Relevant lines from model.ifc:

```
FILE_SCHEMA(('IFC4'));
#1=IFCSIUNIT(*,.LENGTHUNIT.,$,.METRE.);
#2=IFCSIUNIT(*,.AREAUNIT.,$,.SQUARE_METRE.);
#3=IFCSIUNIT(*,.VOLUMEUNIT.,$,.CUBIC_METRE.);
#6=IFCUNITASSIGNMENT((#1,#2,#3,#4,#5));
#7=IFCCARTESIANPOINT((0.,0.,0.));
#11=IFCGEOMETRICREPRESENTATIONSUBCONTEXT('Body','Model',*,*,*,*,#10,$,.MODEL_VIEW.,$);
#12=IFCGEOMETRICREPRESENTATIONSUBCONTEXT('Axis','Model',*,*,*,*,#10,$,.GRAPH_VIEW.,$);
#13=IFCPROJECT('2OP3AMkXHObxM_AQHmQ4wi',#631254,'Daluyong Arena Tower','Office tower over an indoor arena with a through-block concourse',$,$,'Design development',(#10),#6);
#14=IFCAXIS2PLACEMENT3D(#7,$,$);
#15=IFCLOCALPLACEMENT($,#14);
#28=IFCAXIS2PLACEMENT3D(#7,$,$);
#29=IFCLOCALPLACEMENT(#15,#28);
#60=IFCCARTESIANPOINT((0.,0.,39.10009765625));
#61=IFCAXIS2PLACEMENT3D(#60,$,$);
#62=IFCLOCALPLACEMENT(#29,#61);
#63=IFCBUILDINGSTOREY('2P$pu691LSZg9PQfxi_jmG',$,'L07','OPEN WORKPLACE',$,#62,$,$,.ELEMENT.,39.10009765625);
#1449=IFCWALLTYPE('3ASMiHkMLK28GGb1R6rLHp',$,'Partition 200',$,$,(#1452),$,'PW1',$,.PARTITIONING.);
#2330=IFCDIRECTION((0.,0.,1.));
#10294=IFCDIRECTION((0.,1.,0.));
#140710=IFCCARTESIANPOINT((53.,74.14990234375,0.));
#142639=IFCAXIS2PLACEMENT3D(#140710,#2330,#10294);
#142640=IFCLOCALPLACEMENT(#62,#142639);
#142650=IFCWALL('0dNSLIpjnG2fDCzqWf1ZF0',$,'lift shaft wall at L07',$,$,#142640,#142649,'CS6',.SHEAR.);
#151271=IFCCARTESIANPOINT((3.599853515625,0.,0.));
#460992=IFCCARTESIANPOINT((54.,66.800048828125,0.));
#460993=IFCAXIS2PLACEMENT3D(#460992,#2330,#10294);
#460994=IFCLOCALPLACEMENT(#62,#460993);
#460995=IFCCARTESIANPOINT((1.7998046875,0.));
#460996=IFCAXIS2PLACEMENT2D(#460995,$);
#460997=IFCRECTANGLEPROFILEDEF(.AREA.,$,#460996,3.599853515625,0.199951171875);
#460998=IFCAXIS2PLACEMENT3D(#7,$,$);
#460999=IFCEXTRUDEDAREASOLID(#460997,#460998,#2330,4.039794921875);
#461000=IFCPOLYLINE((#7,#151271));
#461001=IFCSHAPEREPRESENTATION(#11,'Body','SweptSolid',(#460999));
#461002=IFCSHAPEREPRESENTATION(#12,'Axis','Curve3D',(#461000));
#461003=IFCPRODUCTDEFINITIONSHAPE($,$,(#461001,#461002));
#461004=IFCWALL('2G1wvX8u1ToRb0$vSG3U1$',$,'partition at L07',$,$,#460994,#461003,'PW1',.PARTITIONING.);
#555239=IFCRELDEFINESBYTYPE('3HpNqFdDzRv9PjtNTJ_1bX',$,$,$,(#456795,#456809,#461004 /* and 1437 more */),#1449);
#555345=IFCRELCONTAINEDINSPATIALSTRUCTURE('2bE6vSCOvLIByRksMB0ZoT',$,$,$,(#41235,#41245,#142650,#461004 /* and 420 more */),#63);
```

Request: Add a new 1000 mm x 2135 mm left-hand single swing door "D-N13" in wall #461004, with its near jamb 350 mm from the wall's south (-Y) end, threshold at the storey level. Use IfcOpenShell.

```python
import numpy as np
import ifcopenshell
import ifcopenshell.api.feature
import ifcopenshell.api.geometry
import ifcopenshell.api.root
import ifcopenshell.api.spatial
import ifcopenshell.geom
import ifcopenshell.util.element
import ifcopenshell.util.placement
import ifcopenshell.util.representation
import ifcopenshell.util.shape
import ifcopenshell.util.unit

model = ifcopenshell.open("model.ifc")
unit_scale = ifcopenshell.util.unit.calculate_unit_scale(model)
settings = ifcopenshell.geom.settings()


def volume(element):
    """Net volume in cubic metres, openings subtracted."""
    shape = ifcopenshell.geom.create_shape(settings, element)
    return ifcopenshell.util.shape.get_volume(shape.geometry)


wall = model.by_guid("2G1wvX8u1ToRb0$vSG3U1$")
storey = ifcopenshell.util.element.get_container(wall, ifc_class="IfcBuildingStorey")
context = ifcopenshell.util.representation.get_context(model, "Model", "Body", "MODEL_VIEW")
before = volume(wall)

width, height, from_end, sill = 1, 2.135, 0.35, 0.0  # metres

# The wall runs along its own X axis, and the end named is its -X end.
wall_shape = ifcopenshell.geom.create_shape(settings, wall)
x, y, z = ifcopenshell.util.shape.get_vertices(wall_shape.geometry).T
start = x.min() + from_end
face, thickness = float(y.min()), float(y.max() - y.min())
wall_matrix = ifcopenshell.util.placement.get_local_placement(wall.ObjectPlacement)
level = ifcopenshell.util.placement.get_local_placement(storey.ObjectPlacement)[2, 3]


def in_wall(x, y):
    """Placement at x, y metres in the wall's axes, at sill height."""
    matrix = wall_matrix.copy()
    matrix[:, 3] = wall_matrix @ np.array([x / unit_scale, y / unit_scale, 0.0, 1.0])
    matrix[2, 3] = level + sill / unit_scale
    return matrix


# Opening: a box that overshoots both wall faces by 50 mm.
opening = ifcopenshell.api.root.create_entity(model, ifc_class="IfcOpeningElement", predefined_type="OPENING")
box = ifcopenshell.api.geometry.add_wall_representation(
    model, context=context, length=width, height=height, thickness=thickness + 0.1
)
ifcopenshell.api.geometry.assign_representation(model, product=opening, representation=box)
ifcopenshell.api.geometry.edit_object_placement(model, product=opening, matrix=in_wall(start, face - 0.05), is_si=False)
ifcopenshell.api.feature.add_feature(model, feature=opening, element=wall)

door = ifcopenshell.api.root.create_entity(model, ifc_class="IfcDoor", name="D-N13", predefined_type="DOOR")
door.OverallWidth, door.OverallHeight = width / unit_scale, height / unit_scale
door.OperationType = "SINGLE_SWING_LEFT"
body = ifcopenshell.api.geometry.add_door_representation(
    model,
    context=context,
    overall_width=door.OverallWidth,
    overall_height=door.OverallHeight,
    operation_type="SINGLE_SWING_LEFT",
    lining_properties={"LiningDepth": thickness / unit_scale, "ThresholdDepth": thickness / unit_scale},
)
ifcopenshell.api.geometry.assign_representation(model, product=door, representation=body)
ifcopenshell.api.spatial.assign_container(model, products=[door], relating_structure=storey)
ifcopenshell.api.feature.add_filling(model, opening=opening, element=door)

# The lining spans the wall, so the door starts at the wall face.
ifcopenshell.api.geometry.edit_object_placement(model, product=door, matrix=in_wall(start, face), is_si=False)

after = volume(wall)

print(f"wall volume {before:.3f} -> {after:.3f} m3")

model.write("model_v2.ifc")
```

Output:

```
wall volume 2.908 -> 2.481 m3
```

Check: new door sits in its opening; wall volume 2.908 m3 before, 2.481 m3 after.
